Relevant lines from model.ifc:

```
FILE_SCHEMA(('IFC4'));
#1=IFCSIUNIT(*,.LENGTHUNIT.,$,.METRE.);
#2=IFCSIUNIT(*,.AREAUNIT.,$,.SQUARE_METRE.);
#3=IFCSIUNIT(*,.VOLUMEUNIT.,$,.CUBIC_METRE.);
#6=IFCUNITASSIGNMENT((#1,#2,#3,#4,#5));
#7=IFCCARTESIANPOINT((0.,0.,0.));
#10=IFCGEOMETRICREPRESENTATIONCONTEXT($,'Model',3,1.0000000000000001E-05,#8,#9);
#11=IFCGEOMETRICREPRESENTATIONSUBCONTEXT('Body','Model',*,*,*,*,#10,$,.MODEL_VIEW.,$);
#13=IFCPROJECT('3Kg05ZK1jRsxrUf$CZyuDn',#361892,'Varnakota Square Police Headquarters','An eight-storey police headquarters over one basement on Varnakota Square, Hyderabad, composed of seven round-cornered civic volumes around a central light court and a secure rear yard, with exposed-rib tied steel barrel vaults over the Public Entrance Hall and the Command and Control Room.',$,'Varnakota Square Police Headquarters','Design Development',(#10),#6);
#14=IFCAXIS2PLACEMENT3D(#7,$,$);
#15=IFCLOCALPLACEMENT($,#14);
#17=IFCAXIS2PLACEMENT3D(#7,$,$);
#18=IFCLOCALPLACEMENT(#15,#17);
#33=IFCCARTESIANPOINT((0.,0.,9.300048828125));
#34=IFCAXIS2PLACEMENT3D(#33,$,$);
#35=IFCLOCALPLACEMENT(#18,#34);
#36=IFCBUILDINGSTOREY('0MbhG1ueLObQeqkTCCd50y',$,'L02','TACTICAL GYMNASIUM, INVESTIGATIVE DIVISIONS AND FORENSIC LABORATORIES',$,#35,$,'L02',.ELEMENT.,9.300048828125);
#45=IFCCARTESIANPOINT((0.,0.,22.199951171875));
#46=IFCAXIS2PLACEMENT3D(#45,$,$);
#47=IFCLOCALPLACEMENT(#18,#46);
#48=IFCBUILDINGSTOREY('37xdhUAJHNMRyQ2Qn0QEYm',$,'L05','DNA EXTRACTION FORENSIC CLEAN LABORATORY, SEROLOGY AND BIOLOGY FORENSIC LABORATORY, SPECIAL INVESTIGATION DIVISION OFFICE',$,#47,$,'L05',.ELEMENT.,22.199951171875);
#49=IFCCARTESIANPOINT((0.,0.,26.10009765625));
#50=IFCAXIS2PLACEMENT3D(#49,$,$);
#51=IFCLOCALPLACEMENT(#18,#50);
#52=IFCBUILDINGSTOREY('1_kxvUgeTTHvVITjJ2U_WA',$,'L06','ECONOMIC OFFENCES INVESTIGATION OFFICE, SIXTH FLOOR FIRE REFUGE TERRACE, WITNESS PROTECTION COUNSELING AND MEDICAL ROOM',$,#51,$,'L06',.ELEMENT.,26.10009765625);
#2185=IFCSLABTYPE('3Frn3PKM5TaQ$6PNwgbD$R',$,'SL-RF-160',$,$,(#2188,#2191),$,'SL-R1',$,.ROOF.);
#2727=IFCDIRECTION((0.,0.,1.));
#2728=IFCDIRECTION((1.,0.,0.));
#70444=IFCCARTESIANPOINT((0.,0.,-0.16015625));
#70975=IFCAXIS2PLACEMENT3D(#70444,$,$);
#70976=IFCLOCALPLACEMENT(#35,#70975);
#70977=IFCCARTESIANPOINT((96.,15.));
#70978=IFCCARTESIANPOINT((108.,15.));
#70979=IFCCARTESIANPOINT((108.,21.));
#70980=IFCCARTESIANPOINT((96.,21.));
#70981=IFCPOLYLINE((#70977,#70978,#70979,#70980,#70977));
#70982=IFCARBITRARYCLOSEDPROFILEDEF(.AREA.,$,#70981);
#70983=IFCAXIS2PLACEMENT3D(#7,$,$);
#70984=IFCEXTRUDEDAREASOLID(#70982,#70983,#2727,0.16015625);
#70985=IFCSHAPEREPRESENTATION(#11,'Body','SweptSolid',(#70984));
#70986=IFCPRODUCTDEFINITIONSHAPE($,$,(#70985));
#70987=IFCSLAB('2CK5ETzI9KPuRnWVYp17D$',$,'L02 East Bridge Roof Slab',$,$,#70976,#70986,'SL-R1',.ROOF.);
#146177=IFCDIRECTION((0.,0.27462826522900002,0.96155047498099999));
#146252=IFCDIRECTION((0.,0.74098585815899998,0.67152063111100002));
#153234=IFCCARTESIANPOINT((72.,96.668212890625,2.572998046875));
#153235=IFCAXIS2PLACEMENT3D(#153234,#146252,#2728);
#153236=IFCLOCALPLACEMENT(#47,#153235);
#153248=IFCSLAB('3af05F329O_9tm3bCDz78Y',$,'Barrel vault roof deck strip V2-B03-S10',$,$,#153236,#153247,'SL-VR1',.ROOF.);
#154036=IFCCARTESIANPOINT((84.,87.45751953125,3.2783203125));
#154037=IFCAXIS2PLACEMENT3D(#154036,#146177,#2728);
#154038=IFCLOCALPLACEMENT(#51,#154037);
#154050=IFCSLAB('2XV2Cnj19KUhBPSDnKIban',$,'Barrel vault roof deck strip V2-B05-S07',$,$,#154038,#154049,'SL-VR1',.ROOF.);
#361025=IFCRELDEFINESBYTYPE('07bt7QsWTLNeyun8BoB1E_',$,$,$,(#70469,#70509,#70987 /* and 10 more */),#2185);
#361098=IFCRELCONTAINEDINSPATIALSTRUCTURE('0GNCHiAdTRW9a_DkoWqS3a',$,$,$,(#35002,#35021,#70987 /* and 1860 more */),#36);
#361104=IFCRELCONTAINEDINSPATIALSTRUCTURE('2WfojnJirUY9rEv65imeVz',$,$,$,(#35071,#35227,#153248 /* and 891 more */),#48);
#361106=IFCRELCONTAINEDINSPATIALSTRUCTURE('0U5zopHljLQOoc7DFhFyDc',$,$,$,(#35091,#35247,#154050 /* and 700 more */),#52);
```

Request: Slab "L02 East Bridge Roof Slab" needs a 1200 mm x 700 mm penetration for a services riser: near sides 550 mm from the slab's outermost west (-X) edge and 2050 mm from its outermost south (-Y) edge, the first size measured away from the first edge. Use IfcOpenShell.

```python
import numpy as np
import ifcopenshell
import ifcopenshell.api.feature
import ifcopenshell.api.geometry
import ifcopenshell.api.root
import ifcopenshell.geom
import ifcopenshell.util.placement
import ifcopenshell.util.representation
import ifcopenshell.util.shape
import ifcopenshell.util.unit

model = ifcopenshell.open("model.ifc")
unit_scale = ifcopenshell.util.unit.calculate_unit_scale(model)
settings = ifcopenshell.geom.settings()


def volume(element):
    """Net volume in cubic metres, openings subtracted."""
    shape = ifcopenshell.geom.create_shape(settings, element)
    return ifcopenshell.util.shape.get_volume(shape.geometry)


slab = model.by_guid("2CK5ETzI9KPuRnWVYp17D$")
before = volume(slab)

# Extent in the slab's own axes, in metres. The edges named are its -X and -Y sides.
slab_shape = ifcopenshell.geom.create_shape(settings, slab)
vertices = ifcopenshell.util.shape.get_vertices(slab_shape.geometry)
x_min, y_min, bottom = vertices.min(axis=0)
top = vertices[:, 2].max()

opening = ifcopenshell.api.root.create_entity(model, ifc_class="IfcOpeningElement", name="Services riser opening", predefined_type="OPENING")
context = ifcopenshell.util.representation.get_context(model, "Model", "Body", "MODEL_VIEW")
width, depth = 1.2, 0.7
outline = [(0.0, 0.0), (width, 0.0), (width, depth), (0.0, depth), (0.0, 0.0)]
# Overshoot both faces by 50 mm so the cut is clean.
shape = ifcopenshell.api.geometry.add_slab_representation(
    model, context=context, depth=top - bottom + 0.1, polyline=outline
)
ifcopenshell.api.geometry.assign_representation(model, product=opening, representation=shape)

matrix = ifcopenshell.util.placement.get_local_placement(slab.ObjectPlacement)
matrix[:, 3] = matrix @ np.append(np.array([x_min + 0.55, y_min + 2.05, bottom - 0.05]) / unit_scale, 1.0)
ifcopenshell.api.geometry.edit_object_placement(model, product=opening, matrix=matrix, is_si=False)
ifcopenshell.api.feature.add_feature(model, feature=opening, element=slab)

after = volume(slab)

print(f"slab volume {before:.3f} -> {after:.3f} m3")

model.write("model_rev.ifc")
```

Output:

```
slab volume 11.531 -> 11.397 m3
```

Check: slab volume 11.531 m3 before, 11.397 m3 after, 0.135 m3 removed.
